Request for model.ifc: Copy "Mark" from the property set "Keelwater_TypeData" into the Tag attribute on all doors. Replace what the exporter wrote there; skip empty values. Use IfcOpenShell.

First a look at what the model holds.

```python
import ifcopenshell
import ifcopenshell.util.element

model = ifcopenshell.open("model.ifc")
print(model.schema)
doors = model.by_type("IfcDoor")
print(len(doors), "doors")
for e in doors[:8]:
    source = ifcopenshell.util.element.get_pset(e, "Keelwater_TypeData", "Mark")
    target = e.Tag
    print(e.id(), repr(source), repr(target), sep=" | ")
```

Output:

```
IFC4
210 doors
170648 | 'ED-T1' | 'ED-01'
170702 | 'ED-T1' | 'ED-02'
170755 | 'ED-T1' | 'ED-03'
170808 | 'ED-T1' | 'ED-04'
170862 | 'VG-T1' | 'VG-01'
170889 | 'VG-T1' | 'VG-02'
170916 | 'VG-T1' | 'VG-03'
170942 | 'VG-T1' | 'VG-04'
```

```python
import ifcopenshell
import ifcopenshell.util.element

model = ifcopenshell.open("model.ifc")

count = 0
for e in model.by_type("IfcDoor"):
    value = ifcopenshell.util.element.get_pset(e, "Keelwater_TypeData", "Mark")
    current = e.Tag
    if not value or not value.strip() or current == value:
        continue
    e.Tag = value
    count += 1

print(count, "doors updated")

model.write("model-out.ifc")
```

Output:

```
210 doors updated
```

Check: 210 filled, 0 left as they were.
